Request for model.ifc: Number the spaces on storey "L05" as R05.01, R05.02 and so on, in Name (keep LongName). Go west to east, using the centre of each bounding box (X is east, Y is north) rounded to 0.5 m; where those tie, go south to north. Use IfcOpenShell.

First a look at what the model holds.

```python
import ifcopenshell
import ifcopenshell.util.element
import ifcopenshell.util.placement

model = ifcopenshell.open("model.ifc")
print(model.schema)
storey = next(s for s in model.by_type("IfcBuildingStorey") if s.Name == "L05")
spaces = [e for e in ifcopenshell.util.element.get_decomposition(storey) if e.is_a("IfcSpace")]
for e in sorted(spaces, key=lambda e: e.id()):
    origin = ifcopenshell.util.placement.get_local_placement(e.ObjectPlacement)[:3, 3]
    print(e.id(), e.Name, e.LongName, origin.round(2) + 0.0, sep=" | ")
```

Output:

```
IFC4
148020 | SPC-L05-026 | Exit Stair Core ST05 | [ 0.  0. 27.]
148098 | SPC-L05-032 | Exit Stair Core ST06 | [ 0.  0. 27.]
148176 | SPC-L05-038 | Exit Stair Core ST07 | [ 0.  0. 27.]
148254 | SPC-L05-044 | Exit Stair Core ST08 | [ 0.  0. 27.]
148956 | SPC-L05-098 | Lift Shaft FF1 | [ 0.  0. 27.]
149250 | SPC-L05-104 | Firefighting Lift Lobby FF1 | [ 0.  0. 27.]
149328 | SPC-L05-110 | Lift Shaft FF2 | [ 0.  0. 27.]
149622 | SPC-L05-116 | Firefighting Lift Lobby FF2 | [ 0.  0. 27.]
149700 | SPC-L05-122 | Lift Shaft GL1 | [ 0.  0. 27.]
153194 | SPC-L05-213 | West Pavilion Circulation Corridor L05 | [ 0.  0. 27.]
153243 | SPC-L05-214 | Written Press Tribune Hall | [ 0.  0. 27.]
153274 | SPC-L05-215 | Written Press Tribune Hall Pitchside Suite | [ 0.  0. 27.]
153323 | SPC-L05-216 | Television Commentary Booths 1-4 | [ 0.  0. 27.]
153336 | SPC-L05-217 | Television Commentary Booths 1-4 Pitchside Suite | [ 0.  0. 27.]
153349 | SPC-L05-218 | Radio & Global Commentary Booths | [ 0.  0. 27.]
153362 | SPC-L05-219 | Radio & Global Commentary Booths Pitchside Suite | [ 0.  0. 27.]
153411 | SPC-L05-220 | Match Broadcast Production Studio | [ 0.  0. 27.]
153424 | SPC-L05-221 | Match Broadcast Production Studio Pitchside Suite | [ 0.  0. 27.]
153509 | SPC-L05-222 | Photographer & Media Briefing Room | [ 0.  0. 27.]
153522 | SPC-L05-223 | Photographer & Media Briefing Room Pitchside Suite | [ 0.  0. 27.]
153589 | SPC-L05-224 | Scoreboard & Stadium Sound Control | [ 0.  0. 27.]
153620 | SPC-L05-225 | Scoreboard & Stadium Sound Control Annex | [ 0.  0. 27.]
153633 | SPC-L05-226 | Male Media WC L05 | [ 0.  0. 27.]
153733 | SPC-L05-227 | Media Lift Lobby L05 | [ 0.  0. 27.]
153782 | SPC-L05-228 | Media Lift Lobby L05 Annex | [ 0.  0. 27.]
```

```python
import ifcopenshell
import ifcopenshell.geom
import ifcopenshell.util.element
import ifcopenshell.util.shape

model = ifcopenshell.open("model.ifc")
settings = ifcopenshell.geom.settings()
settings.set("use-world-coords", True)


def centre(element):
    shape = ifcopenshell.geom.create_shape(settings, element)
    return ifcopenshell.util.shape.get_bbox_centroid(shape.geometry)


storey = next(s for s in model.by_type("IfcBuildingStorey") if s.Name == "L05")
spaces = [e for e in ifcopenshell.util.element.get_decomposition(storey) if e.is_a("IfcSpace")]

# Insertion points can sit at a corner or the storey origin, so sort by the geometry (in metres).
centres = {e: centre(e) for e in spaces}
spaces.sort(key=lambda e: (round(centres[e][0] / 0.5), centres[e][1]))

for i, e in enumerate(spaces, start=1):
    number = f"R05.{i:02d}"
    e.Name = number
    print(e.id(), number)

model.write("model_rev.ifc")
```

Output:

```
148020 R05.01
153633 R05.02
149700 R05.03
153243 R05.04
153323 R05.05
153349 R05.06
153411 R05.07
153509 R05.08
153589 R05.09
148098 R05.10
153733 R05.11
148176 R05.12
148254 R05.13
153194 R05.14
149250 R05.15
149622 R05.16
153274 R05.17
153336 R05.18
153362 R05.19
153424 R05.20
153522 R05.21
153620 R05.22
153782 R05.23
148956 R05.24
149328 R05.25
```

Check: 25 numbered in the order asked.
